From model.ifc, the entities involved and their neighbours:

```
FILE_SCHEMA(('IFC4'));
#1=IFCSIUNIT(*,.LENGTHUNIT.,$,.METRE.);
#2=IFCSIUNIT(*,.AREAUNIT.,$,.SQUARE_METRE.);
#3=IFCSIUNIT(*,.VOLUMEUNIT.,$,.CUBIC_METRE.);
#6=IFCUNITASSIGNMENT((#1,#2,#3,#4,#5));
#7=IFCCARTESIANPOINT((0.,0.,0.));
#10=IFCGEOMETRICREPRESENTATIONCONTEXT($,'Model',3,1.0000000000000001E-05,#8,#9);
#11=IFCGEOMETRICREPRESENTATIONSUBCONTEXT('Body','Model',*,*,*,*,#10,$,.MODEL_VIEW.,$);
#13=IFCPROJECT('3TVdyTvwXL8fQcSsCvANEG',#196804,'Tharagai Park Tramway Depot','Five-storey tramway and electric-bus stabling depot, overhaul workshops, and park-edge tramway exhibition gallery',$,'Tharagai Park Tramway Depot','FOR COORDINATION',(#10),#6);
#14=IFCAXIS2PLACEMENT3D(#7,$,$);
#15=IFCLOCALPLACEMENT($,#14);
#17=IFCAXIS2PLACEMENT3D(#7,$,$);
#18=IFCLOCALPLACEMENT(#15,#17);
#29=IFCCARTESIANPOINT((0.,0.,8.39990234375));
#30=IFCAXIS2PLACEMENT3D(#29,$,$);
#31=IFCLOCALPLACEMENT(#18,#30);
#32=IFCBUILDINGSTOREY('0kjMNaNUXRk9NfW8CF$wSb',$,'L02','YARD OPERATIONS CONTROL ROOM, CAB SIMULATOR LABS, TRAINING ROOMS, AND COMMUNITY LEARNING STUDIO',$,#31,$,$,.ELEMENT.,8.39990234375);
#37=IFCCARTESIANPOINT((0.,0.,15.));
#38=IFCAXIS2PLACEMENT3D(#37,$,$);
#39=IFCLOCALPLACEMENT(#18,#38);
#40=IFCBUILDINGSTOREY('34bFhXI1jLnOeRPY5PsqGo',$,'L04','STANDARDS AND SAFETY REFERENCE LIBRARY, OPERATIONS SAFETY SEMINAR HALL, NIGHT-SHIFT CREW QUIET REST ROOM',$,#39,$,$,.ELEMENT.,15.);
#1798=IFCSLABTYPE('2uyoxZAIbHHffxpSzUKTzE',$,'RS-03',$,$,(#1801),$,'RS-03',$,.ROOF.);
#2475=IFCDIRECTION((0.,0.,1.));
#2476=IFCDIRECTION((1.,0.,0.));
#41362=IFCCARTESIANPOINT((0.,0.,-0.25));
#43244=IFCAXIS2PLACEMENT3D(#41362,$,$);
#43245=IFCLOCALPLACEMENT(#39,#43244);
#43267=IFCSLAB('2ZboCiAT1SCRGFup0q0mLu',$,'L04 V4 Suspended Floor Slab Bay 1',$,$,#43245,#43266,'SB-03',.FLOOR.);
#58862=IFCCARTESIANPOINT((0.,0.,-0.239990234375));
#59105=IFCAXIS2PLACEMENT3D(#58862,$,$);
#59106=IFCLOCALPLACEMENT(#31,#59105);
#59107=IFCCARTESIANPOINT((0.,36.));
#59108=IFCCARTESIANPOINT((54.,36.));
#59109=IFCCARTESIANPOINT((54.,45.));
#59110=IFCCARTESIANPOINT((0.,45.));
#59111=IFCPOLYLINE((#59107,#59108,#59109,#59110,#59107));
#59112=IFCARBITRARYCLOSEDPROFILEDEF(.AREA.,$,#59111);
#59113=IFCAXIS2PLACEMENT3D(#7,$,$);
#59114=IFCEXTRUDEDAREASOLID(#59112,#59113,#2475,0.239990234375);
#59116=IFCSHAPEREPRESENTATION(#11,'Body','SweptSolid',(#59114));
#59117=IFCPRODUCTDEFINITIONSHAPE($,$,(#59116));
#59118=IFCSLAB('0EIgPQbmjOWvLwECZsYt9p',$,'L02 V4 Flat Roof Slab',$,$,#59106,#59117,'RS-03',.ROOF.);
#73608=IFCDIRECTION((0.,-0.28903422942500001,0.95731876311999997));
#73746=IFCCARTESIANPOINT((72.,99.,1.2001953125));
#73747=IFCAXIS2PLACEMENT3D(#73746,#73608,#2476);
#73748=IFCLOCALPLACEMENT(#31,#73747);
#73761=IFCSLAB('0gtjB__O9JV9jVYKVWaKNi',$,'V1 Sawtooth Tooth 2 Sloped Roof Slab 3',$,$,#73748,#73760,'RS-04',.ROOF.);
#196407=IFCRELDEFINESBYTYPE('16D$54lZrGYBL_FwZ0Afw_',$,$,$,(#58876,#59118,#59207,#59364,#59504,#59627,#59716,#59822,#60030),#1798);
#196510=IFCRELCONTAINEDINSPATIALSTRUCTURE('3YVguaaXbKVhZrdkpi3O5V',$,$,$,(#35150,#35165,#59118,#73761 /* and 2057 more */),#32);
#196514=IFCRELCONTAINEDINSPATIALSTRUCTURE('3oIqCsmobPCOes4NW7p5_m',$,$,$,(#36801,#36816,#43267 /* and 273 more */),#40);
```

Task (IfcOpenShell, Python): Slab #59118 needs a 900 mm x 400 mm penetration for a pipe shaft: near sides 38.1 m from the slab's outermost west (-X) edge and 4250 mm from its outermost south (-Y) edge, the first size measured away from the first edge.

```python
import numpy as np
import ifcopenshell
import ifcopenshell.api.feature
import ifcopenshell.api.geometry
import ifcopenshell.api.root
import ifcopenshell.geom
import ifcopenshell.util.placement
import ifcopenshell.util.representation
import ifcopenshell.util.shape
import ifcopenshell.util.unit

model = ifcopenshell.open("model.ifc")
unit_scale = ifcopenshell.util.unit.calculate_unit_scale(model)
settings = ifcopenshell.geom.settings()


def volume(element):
    """Net volume in cubic metres, openings subtracted."""
    shape = ifcopenshell.geom.create_shape(settings, element)
    return ifcopenshell.util.shape.get_volume(shape.geometry)


slab = model.by_guid("0EIgPQbmjOWvLwECZsYt9p")
before = volume(slab)

# Extent in the slab's own axes, in metres. The edges named are its -X and -Y sides.
slab_shape = ifcopenshell.geom.create_shape(settings, slab)
vertices = ifcopenshell.util.shape.get_vertices(slab_shape.geometry)
x_min, y_min, bottom = vertices.min(axis=0)
top = vertices[:, 2].max()

opening = ifcopenshell.api.root.create_entity(model, ifc_class="IfcOpeningElement", name="Pipe shaft opening", predefined_type="OPENING")
context = ifcopenshell.util.representation.get_context(model, "Model", "Body", "MODEL_VIEW")
width, depth = 0.9, 0.4
outline = [(0.0, 0.0), (width, 0.0), (width, depth), (0.0, depth), (0.0, 0.0)]
# Overshoot both faces by 50 mm so the cut is clean.
shape = ifcopenshell.api.geometry.add_slab_representation(
    model, context=context, depth=top - bottom + 0.1, polyline=outline
)
ifcopenshell.api.geometry.assign_representation(model, product=opening, representation=shape)

matrix = ifcopenshell.util.placement.get_local_placement(slab.ObjectPlacement)
matrix[:, 3] = matrix @ np.append(np.array([x_min + 38.1, y_min + 4.25, bottom - 0.05]) / unit_scale, 1.0)
ifcopenshell.api.geometry.edit_object_placement(model, product=opening, matrix=matrix, is_si=False)
ifcopenshell.api.feature.add_feature(model, feature=opening, element=slab)

after = volume(slab)

print(f"slab volume {before:.3f} -> {after:.3f} m3")

model.write("model_v2.ifc")
```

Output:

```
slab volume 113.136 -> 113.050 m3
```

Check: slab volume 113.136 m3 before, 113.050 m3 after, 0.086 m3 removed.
